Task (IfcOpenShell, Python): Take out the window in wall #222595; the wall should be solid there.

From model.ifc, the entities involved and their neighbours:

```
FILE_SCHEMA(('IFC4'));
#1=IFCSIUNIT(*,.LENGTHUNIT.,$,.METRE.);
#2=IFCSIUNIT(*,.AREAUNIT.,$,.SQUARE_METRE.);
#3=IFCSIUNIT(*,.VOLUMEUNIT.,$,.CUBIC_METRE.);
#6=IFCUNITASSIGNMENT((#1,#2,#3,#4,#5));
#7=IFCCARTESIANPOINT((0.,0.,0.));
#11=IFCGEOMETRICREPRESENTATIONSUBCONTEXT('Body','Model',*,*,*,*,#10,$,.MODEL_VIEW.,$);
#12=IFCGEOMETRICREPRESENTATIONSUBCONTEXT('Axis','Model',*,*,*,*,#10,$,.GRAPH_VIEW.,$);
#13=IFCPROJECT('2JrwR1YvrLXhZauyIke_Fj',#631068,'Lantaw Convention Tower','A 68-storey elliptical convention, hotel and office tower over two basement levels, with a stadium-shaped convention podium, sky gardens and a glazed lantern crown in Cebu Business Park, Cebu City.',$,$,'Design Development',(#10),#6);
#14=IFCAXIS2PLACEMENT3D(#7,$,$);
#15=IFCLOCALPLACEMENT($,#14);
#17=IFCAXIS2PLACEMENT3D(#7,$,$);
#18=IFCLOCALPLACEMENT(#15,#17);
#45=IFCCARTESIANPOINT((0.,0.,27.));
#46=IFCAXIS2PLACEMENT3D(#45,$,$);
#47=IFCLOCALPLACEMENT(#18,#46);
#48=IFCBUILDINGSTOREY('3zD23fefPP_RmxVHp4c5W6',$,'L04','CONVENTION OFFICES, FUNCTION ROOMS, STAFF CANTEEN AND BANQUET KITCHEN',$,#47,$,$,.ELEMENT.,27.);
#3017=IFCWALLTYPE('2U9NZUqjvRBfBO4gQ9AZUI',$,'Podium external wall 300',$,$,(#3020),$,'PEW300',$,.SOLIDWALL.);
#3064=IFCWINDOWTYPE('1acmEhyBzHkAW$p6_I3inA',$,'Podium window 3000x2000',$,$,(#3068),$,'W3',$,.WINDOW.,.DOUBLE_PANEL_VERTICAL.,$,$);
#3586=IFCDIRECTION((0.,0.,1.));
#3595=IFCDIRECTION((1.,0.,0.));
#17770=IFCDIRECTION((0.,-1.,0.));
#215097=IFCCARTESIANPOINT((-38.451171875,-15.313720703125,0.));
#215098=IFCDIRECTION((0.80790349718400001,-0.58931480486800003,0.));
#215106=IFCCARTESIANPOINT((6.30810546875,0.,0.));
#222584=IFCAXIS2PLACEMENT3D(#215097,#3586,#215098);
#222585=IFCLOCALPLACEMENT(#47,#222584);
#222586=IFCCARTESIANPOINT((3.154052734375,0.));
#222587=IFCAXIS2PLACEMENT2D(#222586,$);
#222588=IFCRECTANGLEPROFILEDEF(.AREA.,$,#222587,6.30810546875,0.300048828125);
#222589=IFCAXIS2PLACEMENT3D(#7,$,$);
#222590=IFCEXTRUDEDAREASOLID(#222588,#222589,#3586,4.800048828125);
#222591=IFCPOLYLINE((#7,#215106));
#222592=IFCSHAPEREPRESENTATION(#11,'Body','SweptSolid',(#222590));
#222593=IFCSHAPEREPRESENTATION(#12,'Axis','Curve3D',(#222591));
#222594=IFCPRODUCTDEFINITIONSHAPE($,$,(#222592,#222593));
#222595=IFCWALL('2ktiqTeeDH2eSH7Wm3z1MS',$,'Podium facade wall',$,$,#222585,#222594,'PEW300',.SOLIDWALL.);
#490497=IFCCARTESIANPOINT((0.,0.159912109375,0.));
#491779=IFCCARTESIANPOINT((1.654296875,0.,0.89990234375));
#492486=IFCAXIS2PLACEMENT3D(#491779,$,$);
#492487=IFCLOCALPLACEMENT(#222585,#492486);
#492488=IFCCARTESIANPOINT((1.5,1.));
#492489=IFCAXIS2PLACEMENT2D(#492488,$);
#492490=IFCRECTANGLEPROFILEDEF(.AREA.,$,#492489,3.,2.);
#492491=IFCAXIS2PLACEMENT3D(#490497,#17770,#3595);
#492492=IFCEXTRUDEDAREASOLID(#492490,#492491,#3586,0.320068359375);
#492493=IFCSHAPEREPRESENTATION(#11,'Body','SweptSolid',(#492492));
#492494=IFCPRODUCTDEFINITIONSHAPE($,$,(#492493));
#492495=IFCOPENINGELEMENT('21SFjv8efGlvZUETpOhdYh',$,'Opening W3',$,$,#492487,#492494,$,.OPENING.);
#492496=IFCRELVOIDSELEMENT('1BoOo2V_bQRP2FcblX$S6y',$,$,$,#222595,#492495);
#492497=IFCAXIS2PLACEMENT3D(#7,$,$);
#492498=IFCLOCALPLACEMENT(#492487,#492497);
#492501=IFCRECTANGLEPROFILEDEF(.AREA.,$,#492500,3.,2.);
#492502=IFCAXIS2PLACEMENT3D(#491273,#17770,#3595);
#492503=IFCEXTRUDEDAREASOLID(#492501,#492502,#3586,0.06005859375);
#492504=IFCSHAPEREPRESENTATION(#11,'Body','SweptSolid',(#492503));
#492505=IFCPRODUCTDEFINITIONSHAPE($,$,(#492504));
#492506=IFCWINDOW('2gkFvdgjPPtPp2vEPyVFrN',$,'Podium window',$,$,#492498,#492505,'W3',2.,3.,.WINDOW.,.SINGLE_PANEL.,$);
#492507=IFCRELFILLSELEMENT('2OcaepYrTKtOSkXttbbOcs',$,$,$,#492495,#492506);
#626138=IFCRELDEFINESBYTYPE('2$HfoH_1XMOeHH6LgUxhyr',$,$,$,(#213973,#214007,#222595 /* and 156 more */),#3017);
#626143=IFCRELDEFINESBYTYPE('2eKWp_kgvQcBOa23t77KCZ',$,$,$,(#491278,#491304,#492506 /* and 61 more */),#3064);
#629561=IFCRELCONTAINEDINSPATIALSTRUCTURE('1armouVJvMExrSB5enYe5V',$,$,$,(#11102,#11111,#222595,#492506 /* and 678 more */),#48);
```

```python
import ifcopenshell
import ifcopenshell.api.feature
import ifcopenshell.api.root
import ifcopenshell.geom
import ifcopenshell.util.shape

model = ifcopenshell.open("model.ifc")
settings = ifcopenshell.geom.settings()


def volume(element):
    """Net volume in cubic metres, openings subtracted."""
    shape = ifcopenshell.geom.create_shape(settings, element)
    return ifcopenshell.util.shape.get_volume(shape.geometry)


window = model.by_guid("2gkFvdgjPPtPp2vEPyVFrN")
opening = window.FillsVoids[0].RelatingOpeningElement
wall = opening.VoidsElements[0].RelatingBuildingElement
before = volume(wall)

ifcopenshell.api.root.remove_product(model, product=window)
ifcopenshell.api.feature.remove_feature(model, feature=opening)

after = volume(wall)

print(f"wall volume {before:.3f} -> {after:.3f} m3")

model.write("model_v2.ifc")
```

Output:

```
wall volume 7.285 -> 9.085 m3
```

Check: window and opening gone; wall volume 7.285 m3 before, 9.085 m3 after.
